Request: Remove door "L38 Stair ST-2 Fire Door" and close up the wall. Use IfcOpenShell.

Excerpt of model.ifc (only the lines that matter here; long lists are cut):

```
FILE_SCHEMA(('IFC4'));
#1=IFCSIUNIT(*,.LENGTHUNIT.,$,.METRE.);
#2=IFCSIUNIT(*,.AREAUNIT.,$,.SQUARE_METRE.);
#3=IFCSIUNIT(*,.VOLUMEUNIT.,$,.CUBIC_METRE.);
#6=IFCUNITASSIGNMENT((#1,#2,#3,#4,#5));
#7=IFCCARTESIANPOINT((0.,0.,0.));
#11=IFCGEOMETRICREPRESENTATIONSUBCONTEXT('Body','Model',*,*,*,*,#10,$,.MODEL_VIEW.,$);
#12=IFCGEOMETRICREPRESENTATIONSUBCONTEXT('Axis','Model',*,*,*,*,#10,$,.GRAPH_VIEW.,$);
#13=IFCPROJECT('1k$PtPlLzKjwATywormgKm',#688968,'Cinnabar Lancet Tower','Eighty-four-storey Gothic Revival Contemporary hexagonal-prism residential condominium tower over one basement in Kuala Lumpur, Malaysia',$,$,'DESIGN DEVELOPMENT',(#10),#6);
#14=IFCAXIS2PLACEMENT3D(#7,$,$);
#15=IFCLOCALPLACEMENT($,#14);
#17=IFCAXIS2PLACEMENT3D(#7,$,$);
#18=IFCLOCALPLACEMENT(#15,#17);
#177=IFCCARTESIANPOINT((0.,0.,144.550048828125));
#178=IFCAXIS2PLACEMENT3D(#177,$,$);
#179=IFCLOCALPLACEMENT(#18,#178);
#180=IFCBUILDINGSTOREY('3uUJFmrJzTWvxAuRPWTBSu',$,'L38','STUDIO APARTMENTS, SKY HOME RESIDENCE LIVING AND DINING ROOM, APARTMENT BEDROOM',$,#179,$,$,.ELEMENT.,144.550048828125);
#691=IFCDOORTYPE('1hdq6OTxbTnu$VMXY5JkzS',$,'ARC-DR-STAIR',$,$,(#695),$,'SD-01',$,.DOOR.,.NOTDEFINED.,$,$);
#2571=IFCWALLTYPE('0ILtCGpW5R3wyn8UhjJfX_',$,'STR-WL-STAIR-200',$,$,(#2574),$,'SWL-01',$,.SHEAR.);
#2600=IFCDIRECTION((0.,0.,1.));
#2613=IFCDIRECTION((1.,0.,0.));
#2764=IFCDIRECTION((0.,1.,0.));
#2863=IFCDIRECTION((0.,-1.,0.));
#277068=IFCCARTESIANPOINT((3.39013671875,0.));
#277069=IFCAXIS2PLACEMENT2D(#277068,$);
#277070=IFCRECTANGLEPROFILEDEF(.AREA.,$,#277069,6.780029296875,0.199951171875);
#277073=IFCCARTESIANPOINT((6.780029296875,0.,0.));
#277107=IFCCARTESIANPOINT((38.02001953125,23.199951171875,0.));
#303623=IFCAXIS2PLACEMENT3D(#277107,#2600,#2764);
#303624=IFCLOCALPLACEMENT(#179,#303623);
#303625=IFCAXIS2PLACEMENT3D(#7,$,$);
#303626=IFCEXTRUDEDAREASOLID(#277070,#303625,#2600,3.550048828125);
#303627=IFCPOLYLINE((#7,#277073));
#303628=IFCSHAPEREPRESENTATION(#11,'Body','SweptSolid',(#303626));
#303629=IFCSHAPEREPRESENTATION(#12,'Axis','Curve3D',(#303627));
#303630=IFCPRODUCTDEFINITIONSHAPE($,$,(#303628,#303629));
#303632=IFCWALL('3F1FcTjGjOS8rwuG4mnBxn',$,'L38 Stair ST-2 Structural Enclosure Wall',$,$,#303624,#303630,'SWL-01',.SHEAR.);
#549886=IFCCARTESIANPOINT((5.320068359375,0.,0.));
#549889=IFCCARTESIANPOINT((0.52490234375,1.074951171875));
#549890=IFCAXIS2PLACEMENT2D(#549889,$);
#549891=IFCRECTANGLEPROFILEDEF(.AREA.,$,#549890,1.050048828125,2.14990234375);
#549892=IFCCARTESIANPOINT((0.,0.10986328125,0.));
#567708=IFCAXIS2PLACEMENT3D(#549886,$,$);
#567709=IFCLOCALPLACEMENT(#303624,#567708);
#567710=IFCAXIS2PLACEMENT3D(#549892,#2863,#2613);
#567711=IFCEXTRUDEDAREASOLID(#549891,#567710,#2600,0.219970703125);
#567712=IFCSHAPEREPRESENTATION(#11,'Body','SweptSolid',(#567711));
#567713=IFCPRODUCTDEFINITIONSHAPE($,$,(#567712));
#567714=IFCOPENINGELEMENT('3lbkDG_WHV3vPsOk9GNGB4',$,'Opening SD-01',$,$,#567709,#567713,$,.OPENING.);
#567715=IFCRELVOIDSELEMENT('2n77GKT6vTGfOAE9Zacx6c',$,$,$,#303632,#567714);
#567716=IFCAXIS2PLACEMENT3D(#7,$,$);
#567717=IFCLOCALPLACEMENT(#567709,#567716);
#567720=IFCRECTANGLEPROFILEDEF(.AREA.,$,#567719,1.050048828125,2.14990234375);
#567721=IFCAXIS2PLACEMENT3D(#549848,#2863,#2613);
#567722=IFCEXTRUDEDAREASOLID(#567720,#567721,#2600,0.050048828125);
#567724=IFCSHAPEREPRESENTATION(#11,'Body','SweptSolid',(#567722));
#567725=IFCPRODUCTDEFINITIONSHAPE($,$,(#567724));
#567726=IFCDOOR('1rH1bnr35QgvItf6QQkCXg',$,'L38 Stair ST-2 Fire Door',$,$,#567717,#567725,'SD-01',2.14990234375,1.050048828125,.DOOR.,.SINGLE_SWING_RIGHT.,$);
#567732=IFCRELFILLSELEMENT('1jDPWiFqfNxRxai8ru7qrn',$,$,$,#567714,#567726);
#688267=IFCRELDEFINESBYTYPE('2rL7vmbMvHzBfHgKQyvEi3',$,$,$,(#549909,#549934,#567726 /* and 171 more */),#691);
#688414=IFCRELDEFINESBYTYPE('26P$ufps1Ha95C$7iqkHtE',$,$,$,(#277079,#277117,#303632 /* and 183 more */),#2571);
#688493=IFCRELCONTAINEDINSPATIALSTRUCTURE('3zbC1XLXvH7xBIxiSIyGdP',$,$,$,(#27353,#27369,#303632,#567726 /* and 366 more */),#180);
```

```python
import ifcopenshell
import ifcopenshell.api.feature
import ifcopenshell.api.root
import ifcopenshell.geom
import ifcopenshell.util.shape

model = ifcopenshell.open("model.ifc")
settings = ifcopenshell.geom.settings()


def volume(element):
    """Net volume in cubic metres, openings subtracted."""
    shape = ifcopenshell.geom.create_shape(settings, element)
    return ifcopenshell.util.shape.get_volume(shape.geometry)


door = model.by_id(567726)
opening = door.FillsVoids[0].RelatingOpeningElement
wall = opening.VoidsElements[0].RelatingBuildingElement
before = volume(wall)

ifcopenshell.api.root.remove_product(model, product=door)
ifcopenshell.api.feature.remove_feature(model, feature=opening)

after = volume(wall)

print(f"wall volume {before:.3f} -> {after:.3f} m3")

model.write("model-out.ifc")
```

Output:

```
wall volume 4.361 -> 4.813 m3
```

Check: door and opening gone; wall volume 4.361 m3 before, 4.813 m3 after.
